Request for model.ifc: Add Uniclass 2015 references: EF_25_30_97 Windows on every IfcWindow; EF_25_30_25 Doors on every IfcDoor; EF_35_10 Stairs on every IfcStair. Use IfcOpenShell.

First a look at what the model holds.

```python
import ifcopenshell

model = ifcopenshell.open("model.ifc")
print(model.schema)
print("classifications:", [c.Name for c in model.by_type("IfcClassification")])
for ifc_class in ("IfcDoor", "IfcRoof", "IfcStair", "IfcWall", "IfcWindow"):
    print(ifc_class, len(model.by_type(ifc_class)))
```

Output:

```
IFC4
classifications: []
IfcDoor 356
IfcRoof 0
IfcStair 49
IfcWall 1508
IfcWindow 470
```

```python
import ifcopenshell
import ifcopenshell.api.classification

model = ifcopenshell.open("model.ifc")

system = ifcopenshell.api.classification.add_classification(model, classification="Uniclass 2015")

codes = {
    "IfcWindow": ("EF_25_30_97", "Windows"),
    "IfcDoor": ("EF_25_30_25", "Doors"),
    "IfcStair": ("EF_35_10", "Stairs"),
}
for ifc_class, (code, name) in codes.items():
    products = model.by_type(ifc_class)
    ifcopenshell.api.classification.add_reference(
        model, products=products, classification=system, identification=code, name=name
    )
    print(code, len(products))

model.write("model_edited.ifc")
```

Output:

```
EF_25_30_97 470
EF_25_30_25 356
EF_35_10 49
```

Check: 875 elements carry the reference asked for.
